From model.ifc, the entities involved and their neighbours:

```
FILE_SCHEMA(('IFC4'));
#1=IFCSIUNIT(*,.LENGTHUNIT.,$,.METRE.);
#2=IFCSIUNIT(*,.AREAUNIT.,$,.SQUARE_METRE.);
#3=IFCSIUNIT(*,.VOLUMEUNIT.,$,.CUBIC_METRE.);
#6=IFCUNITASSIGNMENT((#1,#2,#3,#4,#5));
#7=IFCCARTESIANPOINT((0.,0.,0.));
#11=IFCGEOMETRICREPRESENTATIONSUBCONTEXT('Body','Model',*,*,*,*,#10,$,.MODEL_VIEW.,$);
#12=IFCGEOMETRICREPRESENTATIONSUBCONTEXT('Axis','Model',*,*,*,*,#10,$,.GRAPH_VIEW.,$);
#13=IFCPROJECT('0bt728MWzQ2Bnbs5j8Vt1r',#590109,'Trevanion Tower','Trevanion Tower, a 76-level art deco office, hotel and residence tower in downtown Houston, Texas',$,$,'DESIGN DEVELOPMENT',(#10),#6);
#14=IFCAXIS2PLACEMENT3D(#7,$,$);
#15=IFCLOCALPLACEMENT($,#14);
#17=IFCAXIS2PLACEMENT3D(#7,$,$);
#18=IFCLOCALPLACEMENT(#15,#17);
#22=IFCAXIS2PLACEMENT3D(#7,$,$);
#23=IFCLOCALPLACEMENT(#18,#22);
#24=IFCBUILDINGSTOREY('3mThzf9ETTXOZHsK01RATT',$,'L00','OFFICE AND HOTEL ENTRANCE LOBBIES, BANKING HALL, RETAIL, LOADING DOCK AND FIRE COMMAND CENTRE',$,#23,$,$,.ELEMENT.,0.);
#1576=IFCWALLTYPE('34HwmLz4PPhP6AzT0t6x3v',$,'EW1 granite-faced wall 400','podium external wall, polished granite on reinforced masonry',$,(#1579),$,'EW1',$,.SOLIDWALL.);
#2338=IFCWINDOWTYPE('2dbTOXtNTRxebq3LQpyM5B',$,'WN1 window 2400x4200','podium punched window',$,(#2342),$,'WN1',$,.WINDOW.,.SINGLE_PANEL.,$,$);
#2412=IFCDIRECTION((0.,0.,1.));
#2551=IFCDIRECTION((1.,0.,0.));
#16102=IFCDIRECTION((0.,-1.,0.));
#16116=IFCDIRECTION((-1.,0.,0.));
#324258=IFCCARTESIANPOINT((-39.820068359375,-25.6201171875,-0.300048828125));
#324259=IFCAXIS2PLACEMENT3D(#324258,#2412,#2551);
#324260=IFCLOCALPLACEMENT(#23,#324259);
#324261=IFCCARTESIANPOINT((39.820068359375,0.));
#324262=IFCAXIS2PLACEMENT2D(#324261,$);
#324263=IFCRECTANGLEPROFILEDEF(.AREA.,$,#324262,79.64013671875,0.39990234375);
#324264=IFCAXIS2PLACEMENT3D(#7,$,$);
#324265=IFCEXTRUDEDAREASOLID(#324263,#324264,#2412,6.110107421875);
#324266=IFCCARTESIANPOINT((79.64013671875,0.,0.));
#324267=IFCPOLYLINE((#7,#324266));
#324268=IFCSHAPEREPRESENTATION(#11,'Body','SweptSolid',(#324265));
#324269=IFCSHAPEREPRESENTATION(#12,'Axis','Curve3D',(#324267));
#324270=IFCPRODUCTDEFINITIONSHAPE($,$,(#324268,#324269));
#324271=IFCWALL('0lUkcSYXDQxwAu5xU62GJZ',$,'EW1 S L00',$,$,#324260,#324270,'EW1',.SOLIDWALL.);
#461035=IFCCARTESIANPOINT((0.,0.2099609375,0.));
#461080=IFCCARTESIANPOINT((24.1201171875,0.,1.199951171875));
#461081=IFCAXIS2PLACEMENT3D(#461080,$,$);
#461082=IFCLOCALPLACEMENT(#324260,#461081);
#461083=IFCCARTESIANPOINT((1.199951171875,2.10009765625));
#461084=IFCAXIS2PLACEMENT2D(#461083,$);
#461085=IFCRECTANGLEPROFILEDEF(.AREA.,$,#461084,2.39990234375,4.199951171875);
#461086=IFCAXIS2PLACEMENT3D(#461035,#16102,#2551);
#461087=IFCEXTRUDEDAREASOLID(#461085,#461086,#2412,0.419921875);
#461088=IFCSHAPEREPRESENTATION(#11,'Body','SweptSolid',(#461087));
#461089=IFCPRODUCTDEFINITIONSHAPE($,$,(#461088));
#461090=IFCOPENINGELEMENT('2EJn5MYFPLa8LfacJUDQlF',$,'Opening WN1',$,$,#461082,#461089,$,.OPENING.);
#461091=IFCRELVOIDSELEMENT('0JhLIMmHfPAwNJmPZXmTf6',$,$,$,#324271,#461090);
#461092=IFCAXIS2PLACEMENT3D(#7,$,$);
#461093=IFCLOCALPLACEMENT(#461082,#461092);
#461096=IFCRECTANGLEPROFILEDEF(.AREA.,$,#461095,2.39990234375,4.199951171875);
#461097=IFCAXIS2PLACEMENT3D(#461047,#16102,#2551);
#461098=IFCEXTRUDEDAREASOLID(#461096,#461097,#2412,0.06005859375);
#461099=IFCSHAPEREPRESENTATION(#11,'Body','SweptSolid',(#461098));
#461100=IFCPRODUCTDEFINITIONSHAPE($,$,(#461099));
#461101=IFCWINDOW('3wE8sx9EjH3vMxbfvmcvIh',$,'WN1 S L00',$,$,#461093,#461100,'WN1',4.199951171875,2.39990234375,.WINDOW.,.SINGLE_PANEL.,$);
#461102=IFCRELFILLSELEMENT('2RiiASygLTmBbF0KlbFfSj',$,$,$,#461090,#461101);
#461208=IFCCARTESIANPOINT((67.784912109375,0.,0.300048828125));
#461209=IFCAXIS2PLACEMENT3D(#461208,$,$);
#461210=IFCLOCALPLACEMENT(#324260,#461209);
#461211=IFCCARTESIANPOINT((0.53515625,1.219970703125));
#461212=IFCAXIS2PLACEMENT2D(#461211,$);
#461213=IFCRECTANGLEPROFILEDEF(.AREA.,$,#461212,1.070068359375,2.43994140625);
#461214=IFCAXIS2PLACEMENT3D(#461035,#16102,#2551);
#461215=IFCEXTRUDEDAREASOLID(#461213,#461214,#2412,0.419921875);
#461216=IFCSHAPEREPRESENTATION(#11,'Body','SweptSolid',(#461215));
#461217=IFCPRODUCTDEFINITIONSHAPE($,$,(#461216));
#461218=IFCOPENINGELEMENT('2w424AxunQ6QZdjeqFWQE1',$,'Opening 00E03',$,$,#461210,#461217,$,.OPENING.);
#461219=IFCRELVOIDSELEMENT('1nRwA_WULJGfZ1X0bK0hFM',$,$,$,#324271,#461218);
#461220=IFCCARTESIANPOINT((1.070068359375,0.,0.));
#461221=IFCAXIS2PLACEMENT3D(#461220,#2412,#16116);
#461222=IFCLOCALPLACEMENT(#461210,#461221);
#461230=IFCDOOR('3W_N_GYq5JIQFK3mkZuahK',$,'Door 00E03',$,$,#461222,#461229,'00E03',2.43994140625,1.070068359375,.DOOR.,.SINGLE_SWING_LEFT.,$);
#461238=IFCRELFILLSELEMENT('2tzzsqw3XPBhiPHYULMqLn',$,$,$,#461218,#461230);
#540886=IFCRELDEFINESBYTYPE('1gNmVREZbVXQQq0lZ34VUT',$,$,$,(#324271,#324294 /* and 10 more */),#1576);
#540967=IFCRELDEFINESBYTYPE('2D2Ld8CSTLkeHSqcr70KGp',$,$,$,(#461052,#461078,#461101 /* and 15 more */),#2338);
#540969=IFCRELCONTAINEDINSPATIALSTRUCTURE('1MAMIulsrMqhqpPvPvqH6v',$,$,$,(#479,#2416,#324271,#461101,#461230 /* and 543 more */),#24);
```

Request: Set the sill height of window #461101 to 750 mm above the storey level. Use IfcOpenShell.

```python
import numpy as np
import ifcopenshell
import ifcopenshell.api.geometry
import ifcopenshell.geom
import ifcopenshell.util.element
import ifcopenshell.util.placement
import ifcopenshell.util.shape
import ifcopenshell.util.unit

model = ifcopenshell.open("model.ifc")
unit_scale = ifcopenshell.util.unit.calculate_unit_scale(model)

window = model.by_id(461101)
opening = window.FillsVoids[0].RelatingOpeningElement
storey = ifcopenshell.util.element.get_container(window, ifc_class="IfcBuildingStorey")
level = ifcopenshell.util.placement.get_local_placement(storey.ObjectPlacement)[2, 3]

# The opening's origin need not be at the sill, so measure its lowest point.
shape = ifcopenshell.geom.create_shape(ifcopenshell.geom.settings(), opening)
bottom = ifcopenshell.util.shape.get_shape_bottom_elevation(shape, shape.geometry) / unit_scale
dz = level + 0.75 / unit_scale - bottom

shift = np.array([0.0, 0.0, dz])
# The window is placed relative to its opening, so it follows when the opening moves.
matrix = ifcopenshell.util.placement.get_local_placement(opening.ObjectPlacement)
matrix[:3, 3] += shift
ifcopenshell.api.geometry.edit_object_placement(
    model, product=opening, matrix=matrix, is_si=False, should_transform_children=True
)

print(f"moved by {dz * unit_scale:+.3f} m")

model.write("model-out.ifc")
```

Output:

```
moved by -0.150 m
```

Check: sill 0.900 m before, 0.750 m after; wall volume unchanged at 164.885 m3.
